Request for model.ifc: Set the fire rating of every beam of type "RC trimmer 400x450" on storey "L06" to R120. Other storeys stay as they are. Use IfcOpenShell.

First a look at what the model holds.

```python
import ifcopenshell
import ifcopenshell.util.element

model = ifcopenshell.open("model.ifc")
print(model.schema)
storey = next(s for s in model.by_type("IfcBuildingStorey") if s.Name == "L06")
beams = [e for e in ifcopenshell.util.element.get_decomposition(storey) if e.is_a("IfcBeam")]
seen = {}
for e in beams:
    element_type = ifcopenshell.util.element.get_type(e)
    key = (element_type.Name if element_type != e and element_type else None, ifcopenshell.util.element.get_pset(e, "Pset_BeamCommon", "FireRating"))
    seen[key] = seen.get(key, 0) + 1
for (name, value), count in sorted(seen.items(), key=str):
    print(count, "x", name, "|", value)
```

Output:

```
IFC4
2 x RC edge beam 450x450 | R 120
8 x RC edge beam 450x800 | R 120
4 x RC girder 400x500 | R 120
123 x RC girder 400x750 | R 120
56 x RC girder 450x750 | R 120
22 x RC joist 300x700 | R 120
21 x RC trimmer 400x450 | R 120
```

```python
import ifcopenshell
import ifcopenshell.api.pset
import ifcopenshell.util.element

model = ifcopenshell.open("model.ifc")

storey = next(s for s in model.by_type("IfcBuildingStorey") if s.Name == "L06")
beams = [e for e in ifcopenshell.util.element.get_decomposition(storey) if e.is_a("IfcBeam")]

count = 0
for e in beams:
    element_type = ifcopenshell.util.element.get_type(e)
    if element_type in (None, e) or element_type.Name != "RC trimmer 400x450":
        continue
    # add_pset returns the element's existing set when there is one.
    pset = ifcopenshell.api.pset.add_pset(model, product=e, name="Pset_BeamCommon")
    ifcopenshell.api.pset.edit_pset(model, pset=pset, properties={"FireRating": "R120"})
    count += 1

print(count, "beams updated")

model.write("model_updated.ifc")
```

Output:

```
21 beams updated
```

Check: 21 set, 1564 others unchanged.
